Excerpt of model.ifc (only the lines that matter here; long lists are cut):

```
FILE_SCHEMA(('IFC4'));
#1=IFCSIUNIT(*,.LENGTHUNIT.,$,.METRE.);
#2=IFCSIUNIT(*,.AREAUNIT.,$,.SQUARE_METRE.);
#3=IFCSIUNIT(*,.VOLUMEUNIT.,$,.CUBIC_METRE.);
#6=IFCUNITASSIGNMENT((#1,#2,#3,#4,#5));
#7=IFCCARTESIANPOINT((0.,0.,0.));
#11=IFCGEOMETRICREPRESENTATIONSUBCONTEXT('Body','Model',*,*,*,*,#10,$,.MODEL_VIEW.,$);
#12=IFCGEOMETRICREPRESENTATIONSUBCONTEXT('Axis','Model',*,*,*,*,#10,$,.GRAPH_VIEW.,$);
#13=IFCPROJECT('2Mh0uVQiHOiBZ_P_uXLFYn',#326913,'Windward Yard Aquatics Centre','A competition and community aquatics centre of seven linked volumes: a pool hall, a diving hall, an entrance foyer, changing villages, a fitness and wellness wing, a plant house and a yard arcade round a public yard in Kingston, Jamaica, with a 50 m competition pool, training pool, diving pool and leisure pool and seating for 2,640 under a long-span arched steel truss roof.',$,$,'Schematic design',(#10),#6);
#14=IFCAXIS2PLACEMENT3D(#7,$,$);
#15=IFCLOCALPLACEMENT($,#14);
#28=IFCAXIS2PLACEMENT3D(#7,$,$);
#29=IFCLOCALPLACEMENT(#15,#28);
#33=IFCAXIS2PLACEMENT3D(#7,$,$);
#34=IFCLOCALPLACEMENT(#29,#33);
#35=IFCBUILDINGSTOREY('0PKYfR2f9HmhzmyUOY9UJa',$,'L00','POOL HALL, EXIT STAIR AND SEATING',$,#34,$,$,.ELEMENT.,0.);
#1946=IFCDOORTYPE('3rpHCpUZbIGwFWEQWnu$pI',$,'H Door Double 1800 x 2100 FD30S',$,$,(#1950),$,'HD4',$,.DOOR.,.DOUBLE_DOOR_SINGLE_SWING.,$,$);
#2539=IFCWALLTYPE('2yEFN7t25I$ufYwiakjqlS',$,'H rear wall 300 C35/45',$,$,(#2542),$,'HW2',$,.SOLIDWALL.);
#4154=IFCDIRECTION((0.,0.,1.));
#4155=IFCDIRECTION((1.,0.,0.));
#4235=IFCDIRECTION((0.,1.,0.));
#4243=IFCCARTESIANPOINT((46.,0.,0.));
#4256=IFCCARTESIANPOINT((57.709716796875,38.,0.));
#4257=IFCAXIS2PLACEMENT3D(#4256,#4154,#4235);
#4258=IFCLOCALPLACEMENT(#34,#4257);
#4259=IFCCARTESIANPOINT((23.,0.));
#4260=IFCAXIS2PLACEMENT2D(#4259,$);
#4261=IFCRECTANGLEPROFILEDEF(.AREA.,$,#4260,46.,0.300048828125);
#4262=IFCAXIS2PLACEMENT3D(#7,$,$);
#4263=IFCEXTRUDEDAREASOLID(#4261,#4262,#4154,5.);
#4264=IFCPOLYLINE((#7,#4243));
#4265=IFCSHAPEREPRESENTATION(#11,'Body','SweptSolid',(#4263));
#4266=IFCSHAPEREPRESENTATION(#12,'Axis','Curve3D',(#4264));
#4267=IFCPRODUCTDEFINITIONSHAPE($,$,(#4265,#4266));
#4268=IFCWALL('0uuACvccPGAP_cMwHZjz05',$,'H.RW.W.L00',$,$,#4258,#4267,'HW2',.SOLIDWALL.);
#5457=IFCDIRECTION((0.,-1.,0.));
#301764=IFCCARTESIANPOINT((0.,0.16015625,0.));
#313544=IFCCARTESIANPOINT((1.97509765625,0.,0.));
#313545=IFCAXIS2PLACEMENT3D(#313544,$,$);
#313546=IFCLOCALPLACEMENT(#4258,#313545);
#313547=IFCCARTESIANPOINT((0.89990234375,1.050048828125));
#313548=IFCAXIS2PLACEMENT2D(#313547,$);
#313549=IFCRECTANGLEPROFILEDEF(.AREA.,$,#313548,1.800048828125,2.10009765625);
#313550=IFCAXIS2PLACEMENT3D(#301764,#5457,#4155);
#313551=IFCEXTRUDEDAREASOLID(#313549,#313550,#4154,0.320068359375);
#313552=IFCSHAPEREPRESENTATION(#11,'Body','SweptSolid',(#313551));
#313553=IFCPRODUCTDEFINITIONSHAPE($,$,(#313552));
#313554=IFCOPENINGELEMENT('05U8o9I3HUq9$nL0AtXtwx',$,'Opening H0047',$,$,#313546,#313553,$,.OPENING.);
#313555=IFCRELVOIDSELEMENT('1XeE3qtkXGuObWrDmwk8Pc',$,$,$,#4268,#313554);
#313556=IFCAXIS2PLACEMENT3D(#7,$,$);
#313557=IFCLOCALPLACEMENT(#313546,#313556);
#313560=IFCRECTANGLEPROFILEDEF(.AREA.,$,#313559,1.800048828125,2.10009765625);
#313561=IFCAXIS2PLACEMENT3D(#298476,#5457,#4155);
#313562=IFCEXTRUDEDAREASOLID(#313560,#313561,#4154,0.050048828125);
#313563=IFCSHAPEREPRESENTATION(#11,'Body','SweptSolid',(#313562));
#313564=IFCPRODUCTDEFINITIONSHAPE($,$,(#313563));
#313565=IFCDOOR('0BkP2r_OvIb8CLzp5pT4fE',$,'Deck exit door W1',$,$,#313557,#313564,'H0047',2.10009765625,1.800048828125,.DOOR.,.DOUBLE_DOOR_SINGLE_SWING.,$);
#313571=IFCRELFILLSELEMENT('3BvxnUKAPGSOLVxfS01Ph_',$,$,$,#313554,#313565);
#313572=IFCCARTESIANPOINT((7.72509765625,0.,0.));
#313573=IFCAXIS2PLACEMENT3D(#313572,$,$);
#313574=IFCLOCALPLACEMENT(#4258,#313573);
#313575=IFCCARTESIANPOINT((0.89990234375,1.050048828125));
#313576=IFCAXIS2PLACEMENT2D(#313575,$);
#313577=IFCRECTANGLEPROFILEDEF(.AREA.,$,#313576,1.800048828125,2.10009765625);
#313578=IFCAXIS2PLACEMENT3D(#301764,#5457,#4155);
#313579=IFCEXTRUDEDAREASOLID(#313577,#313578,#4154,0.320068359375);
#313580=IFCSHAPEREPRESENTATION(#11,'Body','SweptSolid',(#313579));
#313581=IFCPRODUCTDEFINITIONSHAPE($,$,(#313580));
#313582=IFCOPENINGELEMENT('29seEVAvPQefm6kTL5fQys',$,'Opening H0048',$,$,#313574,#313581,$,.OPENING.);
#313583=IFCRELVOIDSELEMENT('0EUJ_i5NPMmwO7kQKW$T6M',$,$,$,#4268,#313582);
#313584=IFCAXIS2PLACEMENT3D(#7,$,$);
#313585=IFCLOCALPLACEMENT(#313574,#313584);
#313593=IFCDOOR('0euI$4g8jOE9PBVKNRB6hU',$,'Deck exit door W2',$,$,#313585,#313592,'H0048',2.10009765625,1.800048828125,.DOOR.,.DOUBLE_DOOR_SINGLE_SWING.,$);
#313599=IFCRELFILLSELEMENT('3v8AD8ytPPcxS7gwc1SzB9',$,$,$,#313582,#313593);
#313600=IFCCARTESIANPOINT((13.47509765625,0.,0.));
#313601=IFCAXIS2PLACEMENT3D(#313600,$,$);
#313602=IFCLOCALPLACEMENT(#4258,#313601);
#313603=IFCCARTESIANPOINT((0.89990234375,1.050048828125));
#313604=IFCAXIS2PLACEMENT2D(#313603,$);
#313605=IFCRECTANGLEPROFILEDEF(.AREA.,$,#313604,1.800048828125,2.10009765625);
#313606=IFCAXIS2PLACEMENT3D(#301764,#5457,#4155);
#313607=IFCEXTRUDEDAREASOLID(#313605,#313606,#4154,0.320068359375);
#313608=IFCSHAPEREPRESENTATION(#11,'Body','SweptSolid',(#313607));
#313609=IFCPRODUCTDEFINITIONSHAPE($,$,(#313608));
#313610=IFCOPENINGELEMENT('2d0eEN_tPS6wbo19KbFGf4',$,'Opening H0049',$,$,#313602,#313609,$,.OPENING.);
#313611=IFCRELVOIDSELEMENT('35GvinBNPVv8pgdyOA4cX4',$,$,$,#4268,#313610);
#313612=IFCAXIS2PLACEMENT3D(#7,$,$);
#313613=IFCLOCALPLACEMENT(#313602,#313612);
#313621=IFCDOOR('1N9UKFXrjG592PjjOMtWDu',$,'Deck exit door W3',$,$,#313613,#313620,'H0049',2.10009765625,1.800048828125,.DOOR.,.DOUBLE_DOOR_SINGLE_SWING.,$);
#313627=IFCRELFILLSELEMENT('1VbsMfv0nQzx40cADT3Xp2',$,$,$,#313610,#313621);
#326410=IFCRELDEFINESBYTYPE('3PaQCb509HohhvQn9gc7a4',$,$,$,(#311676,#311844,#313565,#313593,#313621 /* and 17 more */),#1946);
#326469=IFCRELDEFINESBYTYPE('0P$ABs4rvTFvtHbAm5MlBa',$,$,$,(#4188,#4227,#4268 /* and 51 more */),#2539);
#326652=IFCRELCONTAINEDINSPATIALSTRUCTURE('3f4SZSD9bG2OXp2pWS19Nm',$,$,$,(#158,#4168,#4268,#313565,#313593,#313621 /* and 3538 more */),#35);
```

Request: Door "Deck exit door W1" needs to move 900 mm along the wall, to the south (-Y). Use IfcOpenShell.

```python
import ifcopenshell
import ifcopenshell.api.geometry
import ifcopenshell.util.placement
import ifcopenshell.util.unit

model = ifcopenshell.open("model.ifc")
unit_scale = ifcopenshell.util.unit.calculate_unit_scale(model)

door = model.by_id(313565)
opening = door.FillsVoids[0].RelatingOpeningElement
wall = opening.VoidsElements[0].RelatingBuildingElement

wall_matrix = ifcopenshell.util.placement.get_local_placement(wall.ObjectPlacement)
shift = wall_matrix[:3, 0] * -0.9 / unit_scale
before = ifcopenshell.util.placement.get_local_placement(door.ObjectPlacement)[:3, 3].copy()

# The door is placed relative to its opening, so it follows when the opening moves.
matrix = ifcopenshell.util.placement.get_local_placement(opening.ObjectPlacement)
matrix[:3, 3] += shift
ifcopenshell.api.geometry.edit_object_placement(
    model, product=opening, matrix=matrix, is_si=False, should_transform_children=True
)

after = ifcopenshell.util.placement.get_local_placement(door.ObjectPlacement)[:3, 3]
print("door moved by", (after - before).round(3) + 0.0)

model.write("model_v2.ifc")
```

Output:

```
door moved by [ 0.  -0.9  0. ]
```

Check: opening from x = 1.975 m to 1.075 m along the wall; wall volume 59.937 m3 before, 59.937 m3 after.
